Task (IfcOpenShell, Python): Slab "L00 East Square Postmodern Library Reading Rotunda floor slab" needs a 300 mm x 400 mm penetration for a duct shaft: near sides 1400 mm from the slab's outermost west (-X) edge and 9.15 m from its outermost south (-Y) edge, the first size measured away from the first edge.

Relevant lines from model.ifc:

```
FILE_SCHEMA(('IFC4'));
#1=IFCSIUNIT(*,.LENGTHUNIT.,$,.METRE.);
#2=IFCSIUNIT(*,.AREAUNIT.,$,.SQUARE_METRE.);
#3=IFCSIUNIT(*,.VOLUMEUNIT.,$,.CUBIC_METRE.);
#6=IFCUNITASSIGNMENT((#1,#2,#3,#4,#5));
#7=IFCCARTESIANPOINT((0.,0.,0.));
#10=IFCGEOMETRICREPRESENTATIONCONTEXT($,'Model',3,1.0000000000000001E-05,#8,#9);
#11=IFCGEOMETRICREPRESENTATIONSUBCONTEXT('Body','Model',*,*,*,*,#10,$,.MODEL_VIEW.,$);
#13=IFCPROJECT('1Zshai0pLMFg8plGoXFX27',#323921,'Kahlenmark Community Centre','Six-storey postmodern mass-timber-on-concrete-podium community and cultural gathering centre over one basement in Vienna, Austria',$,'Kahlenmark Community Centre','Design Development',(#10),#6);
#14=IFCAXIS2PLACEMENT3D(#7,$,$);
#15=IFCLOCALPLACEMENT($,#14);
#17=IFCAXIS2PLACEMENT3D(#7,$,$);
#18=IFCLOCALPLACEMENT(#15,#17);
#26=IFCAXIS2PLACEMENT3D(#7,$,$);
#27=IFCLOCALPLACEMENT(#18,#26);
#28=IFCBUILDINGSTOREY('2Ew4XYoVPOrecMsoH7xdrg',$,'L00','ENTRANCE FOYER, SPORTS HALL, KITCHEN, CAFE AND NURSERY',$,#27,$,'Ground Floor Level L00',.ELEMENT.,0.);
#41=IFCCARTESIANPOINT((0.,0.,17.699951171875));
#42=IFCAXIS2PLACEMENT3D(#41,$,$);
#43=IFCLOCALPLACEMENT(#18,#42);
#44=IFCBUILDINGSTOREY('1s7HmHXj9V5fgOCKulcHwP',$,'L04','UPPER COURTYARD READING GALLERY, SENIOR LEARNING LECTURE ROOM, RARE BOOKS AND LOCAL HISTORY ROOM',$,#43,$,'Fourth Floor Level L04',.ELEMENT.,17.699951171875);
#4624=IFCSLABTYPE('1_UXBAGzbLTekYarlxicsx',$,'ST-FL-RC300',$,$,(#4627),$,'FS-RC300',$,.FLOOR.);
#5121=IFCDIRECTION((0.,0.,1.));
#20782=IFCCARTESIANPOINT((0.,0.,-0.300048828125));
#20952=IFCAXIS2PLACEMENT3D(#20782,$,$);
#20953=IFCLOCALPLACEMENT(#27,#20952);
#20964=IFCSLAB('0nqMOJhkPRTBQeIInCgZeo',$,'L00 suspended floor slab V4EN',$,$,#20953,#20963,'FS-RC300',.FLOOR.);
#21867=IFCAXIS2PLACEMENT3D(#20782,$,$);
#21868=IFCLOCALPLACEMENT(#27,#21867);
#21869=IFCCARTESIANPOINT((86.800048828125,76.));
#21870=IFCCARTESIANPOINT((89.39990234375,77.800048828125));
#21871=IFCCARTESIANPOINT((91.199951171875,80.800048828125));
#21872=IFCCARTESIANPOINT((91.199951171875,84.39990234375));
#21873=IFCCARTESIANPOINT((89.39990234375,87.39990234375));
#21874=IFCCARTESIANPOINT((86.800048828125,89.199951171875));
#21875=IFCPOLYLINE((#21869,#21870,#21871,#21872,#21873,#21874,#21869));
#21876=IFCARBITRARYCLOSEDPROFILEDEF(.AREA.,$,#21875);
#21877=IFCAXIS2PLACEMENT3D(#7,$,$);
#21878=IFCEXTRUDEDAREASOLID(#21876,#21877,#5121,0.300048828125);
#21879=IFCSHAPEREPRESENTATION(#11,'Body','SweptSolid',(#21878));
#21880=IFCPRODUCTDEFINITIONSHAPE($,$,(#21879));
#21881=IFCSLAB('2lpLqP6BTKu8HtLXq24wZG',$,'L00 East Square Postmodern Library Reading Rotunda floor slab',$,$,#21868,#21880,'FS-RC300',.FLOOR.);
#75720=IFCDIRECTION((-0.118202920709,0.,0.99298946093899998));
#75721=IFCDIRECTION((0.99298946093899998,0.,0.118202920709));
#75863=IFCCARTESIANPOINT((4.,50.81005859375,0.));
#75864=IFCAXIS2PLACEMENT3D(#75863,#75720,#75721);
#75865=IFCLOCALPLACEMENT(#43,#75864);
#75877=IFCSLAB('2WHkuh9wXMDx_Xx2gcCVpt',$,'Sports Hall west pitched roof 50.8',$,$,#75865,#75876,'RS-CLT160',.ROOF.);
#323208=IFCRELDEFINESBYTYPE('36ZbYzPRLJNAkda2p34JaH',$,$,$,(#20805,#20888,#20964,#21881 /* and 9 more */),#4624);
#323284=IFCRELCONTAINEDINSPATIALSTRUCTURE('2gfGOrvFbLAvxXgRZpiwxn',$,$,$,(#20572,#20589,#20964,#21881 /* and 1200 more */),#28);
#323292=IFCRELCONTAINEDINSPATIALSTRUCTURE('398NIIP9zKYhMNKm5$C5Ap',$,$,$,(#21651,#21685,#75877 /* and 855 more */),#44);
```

```python
import numpy as np
import ifcopenshell
import ifcopenshell.api.feature
import ifcopenshell.api.geometry
import ifcopenshell.api.root
import ifcopenshell.geom
import ifcopenshell.util.placement
import ifcopenshell.util.representation
import ifcopenshell.util.shape
import ifcopenshell.util.unit

model = ifcopenshell.open("model.ifc")
unit_scale = ifcopenshell.util.unit.calculate_unit_scale(model)
settings = ifcopenshell.geom.settings()


def volume(element):
    """Net volume in cubic metres, openings subtracted."""
    shape = ifcopenshell.geom.create_shape(settings, element)
    return ifcopenshell.util.shape.get_volume(shape.geometry)


slab = model.by_guid("2lpLqP6BTKu8HtLXq24wZG")
before = volume(slab)

# Extent in the slab's own axes, in metres. The edges named are its -X and -Y sides.
slab_shape = ifcopenshell.geom.create_shape(settings, slab)
vertices = ifcopenshell.util.shape.get_vertices(slab_shape.geometry)
x_min, y_min, bottom = vertices.min(axis=0)
top = vertices[:, 2].max()

opening = ifcopenshell.api.root.create_entity(model, ifc_class="IfcOpeningElement", name="Duct shaft opening", predefined_type="OPENING")
context = ifcopenshell.util.representation.get_context(model, "Model", "Body", "MODEL_VIEW")
width, depth = 0.3, 0.4
outline = [(0.0, 0.0), (width, 0.0), (width, depth), (0.0, depth), (0.0, 0.0)]
# Overshoot both faces by 50 mm so the cut is clean.
shape = ifcopenshell.api.geometry.add_slab_representation(
    model, context=context, depth=top - bottom + 0.1, polyline=outline
)
ifcopenshell.api.geometry.assign_representation(model, product=opening, representation=shape)

matrix = ifcopenshell.util.placement.get_local_placement(slab.ObjectPlacement)
matrix[:, 3] = matrix @ np.append(np.array([x_min + 1.4, y_min + 9.15, bottom - 0.05]) / unit_scale, 1.0)
ifcopenshell.api.geometry.edit_object_placement(model, product=opening, matrix=matrix, is_si=False)
ifcopenshell.api.feature.add_feature(model, feature=opening, element=slab)

after = volume(slab)

print(f"slab volume {before:.3f} -> {after:.3f} m3")

model.write("model_v2.ifc")
```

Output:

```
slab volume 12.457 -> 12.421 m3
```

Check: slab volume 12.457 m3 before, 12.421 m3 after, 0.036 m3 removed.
